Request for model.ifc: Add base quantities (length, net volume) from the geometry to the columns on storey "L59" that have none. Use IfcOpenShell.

First a look at what the model holds.

```python
import ifcopenshell
import ifcopenshell.util.element
import ifcopenshell.util.unit

model = ifcopenshell.open("model.ifc")
print(model.schema)
for unit_type in ("LENGTHUNIT", "AREAUNIT", "VOLUMEUNIT"):
    print(unit_type, ifcopenshell.util.unit.calculate_unit_scale(model, unit_type))
storey = next(s for s in model.by_type("IfcBuildingStorey") if s.Name == "L59")
columns = [e for e in ifcopenshell.util.element.get_decomposition(storey) if e.is_a("IfcColumn")]
for e in sorted(columns, key=lambda e: e.id()):
    print(e.id(), e.is_a(), e.Name, list(ifcopenshell.util.element.get_psets(e, qtos_only=True)), sep=" | ")
```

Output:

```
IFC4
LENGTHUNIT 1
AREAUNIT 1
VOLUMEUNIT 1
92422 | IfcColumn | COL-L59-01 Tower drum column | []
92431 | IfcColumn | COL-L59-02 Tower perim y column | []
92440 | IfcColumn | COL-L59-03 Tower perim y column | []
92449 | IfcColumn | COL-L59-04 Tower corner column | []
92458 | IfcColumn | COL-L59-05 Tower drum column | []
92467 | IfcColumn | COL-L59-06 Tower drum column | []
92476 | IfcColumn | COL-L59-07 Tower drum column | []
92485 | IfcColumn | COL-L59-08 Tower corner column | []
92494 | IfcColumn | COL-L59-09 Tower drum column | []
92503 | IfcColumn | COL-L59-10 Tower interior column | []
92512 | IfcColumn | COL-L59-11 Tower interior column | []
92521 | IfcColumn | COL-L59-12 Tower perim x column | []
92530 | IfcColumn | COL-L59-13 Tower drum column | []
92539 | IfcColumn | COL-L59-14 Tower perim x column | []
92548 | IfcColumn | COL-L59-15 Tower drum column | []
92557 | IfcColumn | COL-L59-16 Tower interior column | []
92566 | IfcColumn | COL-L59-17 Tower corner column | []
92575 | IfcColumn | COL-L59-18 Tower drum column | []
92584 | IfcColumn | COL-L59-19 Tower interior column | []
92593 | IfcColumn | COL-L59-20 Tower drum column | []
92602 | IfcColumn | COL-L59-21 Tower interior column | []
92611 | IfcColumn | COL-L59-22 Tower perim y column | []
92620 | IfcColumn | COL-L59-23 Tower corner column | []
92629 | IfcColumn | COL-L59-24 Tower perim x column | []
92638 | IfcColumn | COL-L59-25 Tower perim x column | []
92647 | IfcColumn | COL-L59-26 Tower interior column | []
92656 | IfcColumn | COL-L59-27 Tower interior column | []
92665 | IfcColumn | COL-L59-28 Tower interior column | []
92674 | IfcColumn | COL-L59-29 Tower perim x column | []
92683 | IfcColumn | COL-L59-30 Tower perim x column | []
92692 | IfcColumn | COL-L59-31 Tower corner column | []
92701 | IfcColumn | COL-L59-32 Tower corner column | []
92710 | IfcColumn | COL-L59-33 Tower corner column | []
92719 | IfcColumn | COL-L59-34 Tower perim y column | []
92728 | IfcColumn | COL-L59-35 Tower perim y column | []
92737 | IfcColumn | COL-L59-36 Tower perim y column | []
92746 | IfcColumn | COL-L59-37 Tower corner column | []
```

```python
import ifcopenshell
import ifcopenshell.api.pset
import ifcopenshell.geom
import ifcopenshell.util.element
import ifcopenshell.util.shape
import ifcopenshell.util.unit

model = ifcopenshell.open("model.ifc")
unit_scale = ifcopenshell.util.unit.calculate_unit_scale(model)
volume_scale = ifcopenshell.util.unit.calculate_unit_scale(model, "VOLUMEUNIT")
settings = ifcopenshell.geom.settings()

storey = next(s for s in model.by_type("IfcBuildingStorey") if s.Name == "L59")
columns = [e for e in ifcopenshell.util.element.get_decomposition(storey) if e.is_a("IfcColumn")]

for e in sorted(columns, key=lambda e: e.id()):
    if ifcopenshell.util.element.get_psets(e, qtos_only=True, should_inherit=False):
        continue
    # Geometry comes back in metres, in the element's own axes.
    shape = ifcopenshell.geom.create_shape(settings, e)
    values = {
        "Length": ifcopenshell.util.shape.get_z(shape.geometry) / unit_scale,
        "NetVolume": ifcopenshell.util.shape.get_volume(shape.geometry) / volume_scale,
    }
    qto = ifcopenshell.api.pset.add_qto(model, product=e, name="Qto_ColumnBaseQuantities")
    ifcopenshell.api.pset.edit_qto(model, qto=qto, properties=values)
    print(e.id(), {k: round(v, 3) for k, v in values.items()})

model.write("model-out.ifc")
```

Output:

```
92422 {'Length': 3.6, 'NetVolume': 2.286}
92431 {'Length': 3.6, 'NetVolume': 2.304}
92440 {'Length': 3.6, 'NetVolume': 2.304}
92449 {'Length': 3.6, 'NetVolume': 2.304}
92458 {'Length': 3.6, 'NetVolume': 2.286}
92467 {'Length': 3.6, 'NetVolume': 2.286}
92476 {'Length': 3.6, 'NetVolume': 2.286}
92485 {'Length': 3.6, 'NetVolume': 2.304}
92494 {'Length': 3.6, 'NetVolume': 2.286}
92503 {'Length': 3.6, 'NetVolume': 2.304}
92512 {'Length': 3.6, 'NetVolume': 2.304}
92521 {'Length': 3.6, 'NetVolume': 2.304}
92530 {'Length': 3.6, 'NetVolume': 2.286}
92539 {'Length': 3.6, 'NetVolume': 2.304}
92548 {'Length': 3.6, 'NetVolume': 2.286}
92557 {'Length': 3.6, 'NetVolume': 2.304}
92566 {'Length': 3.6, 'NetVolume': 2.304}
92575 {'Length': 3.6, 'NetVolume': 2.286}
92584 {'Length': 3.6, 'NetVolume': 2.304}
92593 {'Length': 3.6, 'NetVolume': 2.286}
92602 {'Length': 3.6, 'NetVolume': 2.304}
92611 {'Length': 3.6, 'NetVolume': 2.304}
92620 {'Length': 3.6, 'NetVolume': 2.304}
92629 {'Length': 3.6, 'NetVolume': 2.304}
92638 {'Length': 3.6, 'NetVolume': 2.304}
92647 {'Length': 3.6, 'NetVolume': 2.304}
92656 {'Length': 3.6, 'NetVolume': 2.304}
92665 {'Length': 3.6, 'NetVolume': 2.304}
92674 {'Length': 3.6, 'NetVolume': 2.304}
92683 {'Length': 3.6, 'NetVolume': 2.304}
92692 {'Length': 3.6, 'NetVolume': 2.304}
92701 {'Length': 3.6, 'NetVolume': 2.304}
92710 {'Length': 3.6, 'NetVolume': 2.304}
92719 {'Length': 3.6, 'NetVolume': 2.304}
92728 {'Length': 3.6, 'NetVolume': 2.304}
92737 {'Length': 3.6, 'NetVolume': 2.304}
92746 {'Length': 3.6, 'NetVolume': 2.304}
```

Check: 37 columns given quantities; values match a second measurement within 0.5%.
